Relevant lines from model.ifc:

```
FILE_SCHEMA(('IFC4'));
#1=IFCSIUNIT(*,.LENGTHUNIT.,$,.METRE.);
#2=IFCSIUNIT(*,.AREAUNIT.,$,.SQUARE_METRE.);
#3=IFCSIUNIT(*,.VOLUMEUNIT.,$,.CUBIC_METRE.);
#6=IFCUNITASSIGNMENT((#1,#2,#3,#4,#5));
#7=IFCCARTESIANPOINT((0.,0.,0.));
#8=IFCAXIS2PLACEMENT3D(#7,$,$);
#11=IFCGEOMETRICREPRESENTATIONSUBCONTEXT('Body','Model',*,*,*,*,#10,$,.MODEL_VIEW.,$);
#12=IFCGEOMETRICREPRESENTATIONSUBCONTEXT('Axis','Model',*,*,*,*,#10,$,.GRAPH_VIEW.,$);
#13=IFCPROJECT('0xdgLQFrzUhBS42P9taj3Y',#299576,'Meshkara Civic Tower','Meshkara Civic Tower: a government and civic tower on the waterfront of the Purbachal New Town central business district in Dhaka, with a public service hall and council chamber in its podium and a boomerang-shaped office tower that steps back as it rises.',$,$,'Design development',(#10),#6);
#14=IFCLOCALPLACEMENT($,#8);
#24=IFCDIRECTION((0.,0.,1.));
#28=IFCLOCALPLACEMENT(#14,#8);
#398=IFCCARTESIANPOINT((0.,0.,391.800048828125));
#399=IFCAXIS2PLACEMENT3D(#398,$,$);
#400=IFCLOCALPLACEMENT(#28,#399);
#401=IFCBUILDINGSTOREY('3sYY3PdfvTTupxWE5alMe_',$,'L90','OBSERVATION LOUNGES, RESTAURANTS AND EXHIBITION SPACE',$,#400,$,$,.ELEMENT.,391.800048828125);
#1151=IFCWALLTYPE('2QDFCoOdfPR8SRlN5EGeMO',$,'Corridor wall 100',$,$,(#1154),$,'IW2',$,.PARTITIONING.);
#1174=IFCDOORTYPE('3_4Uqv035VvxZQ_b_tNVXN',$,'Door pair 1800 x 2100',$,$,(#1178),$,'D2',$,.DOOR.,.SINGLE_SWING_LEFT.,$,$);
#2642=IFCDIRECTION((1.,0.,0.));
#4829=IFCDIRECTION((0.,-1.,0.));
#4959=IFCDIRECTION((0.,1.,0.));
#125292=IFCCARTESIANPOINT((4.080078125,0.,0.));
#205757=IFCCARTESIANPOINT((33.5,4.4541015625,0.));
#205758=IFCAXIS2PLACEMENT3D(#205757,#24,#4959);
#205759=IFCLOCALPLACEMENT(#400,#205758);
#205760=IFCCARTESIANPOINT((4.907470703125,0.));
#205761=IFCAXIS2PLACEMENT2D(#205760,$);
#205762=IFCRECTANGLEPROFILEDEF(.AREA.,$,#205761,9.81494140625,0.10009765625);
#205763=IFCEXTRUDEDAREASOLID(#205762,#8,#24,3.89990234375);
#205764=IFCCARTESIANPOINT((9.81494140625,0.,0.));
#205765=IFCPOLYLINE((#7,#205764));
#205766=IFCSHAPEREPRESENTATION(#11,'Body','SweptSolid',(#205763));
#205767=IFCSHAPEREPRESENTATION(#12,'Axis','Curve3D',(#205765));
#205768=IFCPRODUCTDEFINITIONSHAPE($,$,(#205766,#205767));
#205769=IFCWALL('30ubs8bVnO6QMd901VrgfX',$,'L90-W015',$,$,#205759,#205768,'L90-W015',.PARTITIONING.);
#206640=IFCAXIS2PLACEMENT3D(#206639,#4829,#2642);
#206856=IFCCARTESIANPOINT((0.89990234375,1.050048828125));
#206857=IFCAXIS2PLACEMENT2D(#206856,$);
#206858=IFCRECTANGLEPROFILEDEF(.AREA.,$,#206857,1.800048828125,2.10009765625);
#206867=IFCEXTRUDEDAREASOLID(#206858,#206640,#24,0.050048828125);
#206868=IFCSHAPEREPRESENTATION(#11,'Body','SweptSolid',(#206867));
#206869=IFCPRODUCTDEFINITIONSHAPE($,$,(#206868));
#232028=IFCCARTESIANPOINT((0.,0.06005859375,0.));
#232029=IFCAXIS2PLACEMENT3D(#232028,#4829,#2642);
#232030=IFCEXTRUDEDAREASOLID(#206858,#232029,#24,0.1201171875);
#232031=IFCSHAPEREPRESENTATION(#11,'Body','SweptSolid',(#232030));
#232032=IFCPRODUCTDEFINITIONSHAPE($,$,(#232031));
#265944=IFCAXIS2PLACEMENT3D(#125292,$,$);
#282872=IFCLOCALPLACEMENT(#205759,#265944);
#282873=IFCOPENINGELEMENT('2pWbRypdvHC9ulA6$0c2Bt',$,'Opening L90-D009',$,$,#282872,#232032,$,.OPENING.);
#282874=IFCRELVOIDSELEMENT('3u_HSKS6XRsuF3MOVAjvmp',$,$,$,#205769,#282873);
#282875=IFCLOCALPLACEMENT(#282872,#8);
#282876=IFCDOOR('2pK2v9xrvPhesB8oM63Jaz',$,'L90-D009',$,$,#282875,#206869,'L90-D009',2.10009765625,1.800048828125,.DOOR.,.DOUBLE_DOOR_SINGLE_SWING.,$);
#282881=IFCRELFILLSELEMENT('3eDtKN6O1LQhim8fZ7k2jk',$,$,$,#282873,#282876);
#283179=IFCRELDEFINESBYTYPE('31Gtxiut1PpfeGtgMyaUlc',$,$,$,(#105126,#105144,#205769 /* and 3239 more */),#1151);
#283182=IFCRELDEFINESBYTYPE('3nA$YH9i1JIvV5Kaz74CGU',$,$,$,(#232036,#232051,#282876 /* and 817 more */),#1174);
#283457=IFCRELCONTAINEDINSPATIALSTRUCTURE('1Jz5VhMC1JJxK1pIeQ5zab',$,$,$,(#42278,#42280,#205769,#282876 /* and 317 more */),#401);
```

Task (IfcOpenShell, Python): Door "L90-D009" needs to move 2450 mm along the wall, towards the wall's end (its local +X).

```python
import ifcopenshell
import ifcopenshell.api.geometry
import ifcopenshell.util.placement

model = ifcopenshell.open("model.ifc")

door = model.by_guid("2pK2v9xrvPhesB8oM63Jaz")
opening = door.FillsVoids[0].RelatingOpeningElement
wall = opening.VoidsElements[0].RelatingBuildingElement

wall_matrix = ifcopenshell.util.placement.get_local_placement(wall.ObjectPlacement)
shift = wall_matrix[:3, 0] * 2.45
before = ifcopenshell.util.placement.get_local_placement(door.ObjectPlacement)[:3, 3].copy()

# The door is placed relative to its opening, so it follows when the opening moves.
matrix = ifcopenshell.util.placement.get_local_placement(opening.ObjectPlacement)
matrix[:3, 3] += shift
ifcopenshell.api.geometry.edit_object_placement(
    model, product=opening, matrix=matrix, is_si=False, should_transform_children=True
)

after = ifcopenshell.util.placement.get_local_placement(door.ObjectPlacement)[:3, 3]
print("door moved by", (after - before).round(3) + 0.0)

model.write("model_edited.ifc")
```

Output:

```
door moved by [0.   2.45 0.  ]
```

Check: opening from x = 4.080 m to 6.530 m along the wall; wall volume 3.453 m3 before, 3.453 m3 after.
